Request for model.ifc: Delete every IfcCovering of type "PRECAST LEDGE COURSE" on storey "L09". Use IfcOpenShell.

First a look at what the model holds.

```python
import ifcopenshell
import ifcopenshell.util.element

model = ifcopenshell.open("model.ifc")
print(model.schema)
storey = next(s for s in model.by_type("IfcBuildingStorey") if s.Name == "L09")
coverings = [e for e in ifcopenshell.util.element.get_decomposition(storey) if e.is_a("IfcCovering")]
seen = {}
for e in coverings:
    element_type = ifcopenshell.util.element.get_type(e)
    name = element_type.Name if element_type not in (None, e) else None
    seen[name] = seen.get(name, 0) + 1
for name, count in sorted(seen.items(), key=str):
    print(count, "x", name)
```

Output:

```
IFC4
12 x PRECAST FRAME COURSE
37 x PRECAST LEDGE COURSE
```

```python
import ifcopenshell
import ifcopenshell.api.root
import ifcopenshell.util.element

model = ifcopenshell.open("model.ifc")

storey = next(s for s in model.by_type("IfcBuildingStorey") if s.Name == "L09")
coverings = [e for e in ifcopenshell.util.element.get_decomposition(storey) if e.is_a("IfcCovering")]
targets = [e for e in coverings if (t := ifcopenshell.util.element.get_type(e)) not in (None, e) and t.Name == "PRECAST LEDGE COURSE"]

for e in targets:
    ifcopenshell.api.root.remove_product(model, product=e)
print(len(targets), "removed")

model.write("model_updated.ifc")
```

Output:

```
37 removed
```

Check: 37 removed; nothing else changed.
